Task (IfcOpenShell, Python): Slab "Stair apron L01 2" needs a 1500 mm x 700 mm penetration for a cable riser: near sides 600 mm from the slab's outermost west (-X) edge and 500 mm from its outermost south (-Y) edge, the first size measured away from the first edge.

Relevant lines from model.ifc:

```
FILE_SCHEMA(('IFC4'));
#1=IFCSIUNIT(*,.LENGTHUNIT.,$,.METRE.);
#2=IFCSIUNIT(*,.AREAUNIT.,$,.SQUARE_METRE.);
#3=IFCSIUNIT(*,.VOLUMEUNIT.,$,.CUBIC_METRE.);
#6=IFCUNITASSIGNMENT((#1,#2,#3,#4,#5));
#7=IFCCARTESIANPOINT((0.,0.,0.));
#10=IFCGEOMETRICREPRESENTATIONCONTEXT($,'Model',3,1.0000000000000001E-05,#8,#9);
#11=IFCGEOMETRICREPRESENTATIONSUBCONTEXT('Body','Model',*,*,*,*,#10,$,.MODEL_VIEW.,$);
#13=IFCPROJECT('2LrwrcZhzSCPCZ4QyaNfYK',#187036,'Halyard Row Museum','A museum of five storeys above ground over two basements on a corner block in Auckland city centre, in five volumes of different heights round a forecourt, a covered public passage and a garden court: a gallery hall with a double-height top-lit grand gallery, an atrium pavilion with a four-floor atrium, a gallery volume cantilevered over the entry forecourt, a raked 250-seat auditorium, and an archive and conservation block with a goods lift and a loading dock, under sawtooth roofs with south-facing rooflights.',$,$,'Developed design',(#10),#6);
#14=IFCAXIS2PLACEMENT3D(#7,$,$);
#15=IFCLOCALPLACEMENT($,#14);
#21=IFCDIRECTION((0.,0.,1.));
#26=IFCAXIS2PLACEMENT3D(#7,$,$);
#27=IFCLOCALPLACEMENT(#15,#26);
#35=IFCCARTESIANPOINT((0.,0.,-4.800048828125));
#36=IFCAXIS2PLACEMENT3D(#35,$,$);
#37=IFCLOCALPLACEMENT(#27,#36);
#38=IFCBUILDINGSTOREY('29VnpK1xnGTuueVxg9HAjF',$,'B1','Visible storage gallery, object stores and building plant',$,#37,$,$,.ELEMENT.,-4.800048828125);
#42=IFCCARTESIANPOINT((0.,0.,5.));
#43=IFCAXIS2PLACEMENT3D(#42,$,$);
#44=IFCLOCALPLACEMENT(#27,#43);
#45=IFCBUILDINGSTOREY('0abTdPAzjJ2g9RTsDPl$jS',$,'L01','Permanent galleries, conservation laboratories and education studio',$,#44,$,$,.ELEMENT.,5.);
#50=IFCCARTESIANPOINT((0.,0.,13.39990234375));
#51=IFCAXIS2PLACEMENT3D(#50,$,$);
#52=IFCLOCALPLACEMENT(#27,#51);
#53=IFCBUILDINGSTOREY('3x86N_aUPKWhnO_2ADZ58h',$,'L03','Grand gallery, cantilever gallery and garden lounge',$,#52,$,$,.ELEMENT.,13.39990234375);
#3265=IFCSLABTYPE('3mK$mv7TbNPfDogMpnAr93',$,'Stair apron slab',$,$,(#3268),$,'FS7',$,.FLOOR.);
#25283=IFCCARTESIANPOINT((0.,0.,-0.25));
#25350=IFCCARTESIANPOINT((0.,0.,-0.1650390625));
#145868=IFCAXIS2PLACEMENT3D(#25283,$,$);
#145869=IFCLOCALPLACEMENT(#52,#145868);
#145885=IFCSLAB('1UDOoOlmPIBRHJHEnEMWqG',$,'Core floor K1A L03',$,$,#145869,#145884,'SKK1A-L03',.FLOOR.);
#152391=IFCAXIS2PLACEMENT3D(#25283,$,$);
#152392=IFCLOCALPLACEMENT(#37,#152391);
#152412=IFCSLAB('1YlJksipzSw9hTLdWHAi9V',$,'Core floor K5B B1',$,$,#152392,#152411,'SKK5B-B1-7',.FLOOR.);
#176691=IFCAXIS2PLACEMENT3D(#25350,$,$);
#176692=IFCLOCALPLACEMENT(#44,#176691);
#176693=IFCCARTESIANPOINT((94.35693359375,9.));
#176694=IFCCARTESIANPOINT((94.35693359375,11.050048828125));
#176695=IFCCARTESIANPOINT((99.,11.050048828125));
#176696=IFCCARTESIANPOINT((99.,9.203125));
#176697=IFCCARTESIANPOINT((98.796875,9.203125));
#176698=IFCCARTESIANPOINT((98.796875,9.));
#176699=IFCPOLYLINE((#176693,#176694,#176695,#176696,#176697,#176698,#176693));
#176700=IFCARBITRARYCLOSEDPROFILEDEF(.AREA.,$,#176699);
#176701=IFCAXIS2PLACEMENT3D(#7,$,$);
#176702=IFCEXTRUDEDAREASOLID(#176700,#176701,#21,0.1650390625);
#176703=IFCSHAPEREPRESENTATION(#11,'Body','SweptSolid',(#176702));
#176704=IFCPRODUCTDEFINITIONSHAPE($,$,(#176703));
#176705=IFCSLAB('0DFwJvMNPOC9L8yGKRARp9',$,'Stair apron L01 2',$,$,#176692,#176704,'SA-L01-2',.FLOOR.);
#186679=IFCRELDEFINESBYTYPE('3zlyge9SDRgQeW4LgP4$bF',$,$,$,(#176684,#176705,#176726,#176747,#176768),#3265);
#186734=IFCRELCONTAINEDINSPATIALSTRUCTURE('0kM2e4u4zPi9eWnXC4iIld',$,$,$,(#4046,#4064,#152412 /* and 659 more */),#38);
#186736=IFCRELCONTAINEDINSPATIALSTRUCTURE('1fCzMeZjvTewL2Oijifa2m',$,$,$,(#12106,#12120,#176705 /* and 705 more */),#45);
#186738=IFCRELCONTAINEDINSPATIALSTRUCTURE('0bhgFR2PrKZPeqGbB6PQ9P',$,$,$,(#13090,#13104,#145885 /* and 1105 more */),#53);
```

```python
import numpy as np
import ifcopenshell
import ifcopenshell.api.feature
import ifcopenshell.api.geometry
import ifcopenshell.api.root
import ifcopenshell.geom
import ifcopenshell.util.placement
import ifcopenshell.util.representation
import ifcopenshell.util.shape
import ifcopenshell.util.unit

model = ifcopenshell.open("model.ifc")
unit_scale = ifcopenshell.util.unit.calculate_unit_scale(model)
settings = ifcopenshell.geom.settings()


def volume(element):
    """Net volume in cubic metres, openings subtracted."""
    shape = ifcopenshell.geom.create_shape(settings, element)
    return ifcopenshell.util.shape.get_volume(shape.geometry)


slab = model.by_guid("0DFwJvMNPOC9L8yGKRARp9")
before = volume(slab)

# Extent in the slab's own axes, in metres. The edges named are its -X and -Y sides.
slab_shape = ifcopenshell.geom.create_shape(settings, slab)
vertices = ifcopenshell.util.shape.get_vertices(slab_shape.geometry)
x_min, y_min, bottom = vertices.min(axis=0)
top = vertices[:, 2].max()

opening = ifcopenshell.api.root.create_entity(model, ifc_class="IfcOpeningElement", name="Cable riser opening", predefined_type="OPENING")
context = ifcopenshell.util.representation.get_context(model, "Model", "Body", "MODEL_VIEW")
width, depth = 1.5, 0.7
outline = [(0.0, 0.0), (width, 0.0), (width, depth), (0.0, depth), (0.0, 0.0)]
# Overshoot both faces by 50 mm so the cut is clean.
shape = ifcopenshell.api.geometry.add_slab_representation(
    model, context=context, depth=top - bottom + 0.1, polyline=outline
)
ifcopenshell.api.geometry.assign_representation(model, product=opening, representation=shape)

matrix = ifcopenshell.util.placement.get_local_placement(slab.ObjectPlacement)
matrix[:, 3] = matrix @ np.append(np.array([x_min + 0.6, y_min + 0.5, bottom - 0.05]) / unit_scale, 1.0)
ifcopenshell.api.geometry.edit_object_placement(model, product=opening, matrix=matrix, is_si=False)
ifcopenshell.api.feature.add_feature(model, feature=opening, element=slab)

after = volume(slab)

print(f"slab volume {before:.3f} -> {after:.3f} m3")

model.write("model_edited.ifc")
```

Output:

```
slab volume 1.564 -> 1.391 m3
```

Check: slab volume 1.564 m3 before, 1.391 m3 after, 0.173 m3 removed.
